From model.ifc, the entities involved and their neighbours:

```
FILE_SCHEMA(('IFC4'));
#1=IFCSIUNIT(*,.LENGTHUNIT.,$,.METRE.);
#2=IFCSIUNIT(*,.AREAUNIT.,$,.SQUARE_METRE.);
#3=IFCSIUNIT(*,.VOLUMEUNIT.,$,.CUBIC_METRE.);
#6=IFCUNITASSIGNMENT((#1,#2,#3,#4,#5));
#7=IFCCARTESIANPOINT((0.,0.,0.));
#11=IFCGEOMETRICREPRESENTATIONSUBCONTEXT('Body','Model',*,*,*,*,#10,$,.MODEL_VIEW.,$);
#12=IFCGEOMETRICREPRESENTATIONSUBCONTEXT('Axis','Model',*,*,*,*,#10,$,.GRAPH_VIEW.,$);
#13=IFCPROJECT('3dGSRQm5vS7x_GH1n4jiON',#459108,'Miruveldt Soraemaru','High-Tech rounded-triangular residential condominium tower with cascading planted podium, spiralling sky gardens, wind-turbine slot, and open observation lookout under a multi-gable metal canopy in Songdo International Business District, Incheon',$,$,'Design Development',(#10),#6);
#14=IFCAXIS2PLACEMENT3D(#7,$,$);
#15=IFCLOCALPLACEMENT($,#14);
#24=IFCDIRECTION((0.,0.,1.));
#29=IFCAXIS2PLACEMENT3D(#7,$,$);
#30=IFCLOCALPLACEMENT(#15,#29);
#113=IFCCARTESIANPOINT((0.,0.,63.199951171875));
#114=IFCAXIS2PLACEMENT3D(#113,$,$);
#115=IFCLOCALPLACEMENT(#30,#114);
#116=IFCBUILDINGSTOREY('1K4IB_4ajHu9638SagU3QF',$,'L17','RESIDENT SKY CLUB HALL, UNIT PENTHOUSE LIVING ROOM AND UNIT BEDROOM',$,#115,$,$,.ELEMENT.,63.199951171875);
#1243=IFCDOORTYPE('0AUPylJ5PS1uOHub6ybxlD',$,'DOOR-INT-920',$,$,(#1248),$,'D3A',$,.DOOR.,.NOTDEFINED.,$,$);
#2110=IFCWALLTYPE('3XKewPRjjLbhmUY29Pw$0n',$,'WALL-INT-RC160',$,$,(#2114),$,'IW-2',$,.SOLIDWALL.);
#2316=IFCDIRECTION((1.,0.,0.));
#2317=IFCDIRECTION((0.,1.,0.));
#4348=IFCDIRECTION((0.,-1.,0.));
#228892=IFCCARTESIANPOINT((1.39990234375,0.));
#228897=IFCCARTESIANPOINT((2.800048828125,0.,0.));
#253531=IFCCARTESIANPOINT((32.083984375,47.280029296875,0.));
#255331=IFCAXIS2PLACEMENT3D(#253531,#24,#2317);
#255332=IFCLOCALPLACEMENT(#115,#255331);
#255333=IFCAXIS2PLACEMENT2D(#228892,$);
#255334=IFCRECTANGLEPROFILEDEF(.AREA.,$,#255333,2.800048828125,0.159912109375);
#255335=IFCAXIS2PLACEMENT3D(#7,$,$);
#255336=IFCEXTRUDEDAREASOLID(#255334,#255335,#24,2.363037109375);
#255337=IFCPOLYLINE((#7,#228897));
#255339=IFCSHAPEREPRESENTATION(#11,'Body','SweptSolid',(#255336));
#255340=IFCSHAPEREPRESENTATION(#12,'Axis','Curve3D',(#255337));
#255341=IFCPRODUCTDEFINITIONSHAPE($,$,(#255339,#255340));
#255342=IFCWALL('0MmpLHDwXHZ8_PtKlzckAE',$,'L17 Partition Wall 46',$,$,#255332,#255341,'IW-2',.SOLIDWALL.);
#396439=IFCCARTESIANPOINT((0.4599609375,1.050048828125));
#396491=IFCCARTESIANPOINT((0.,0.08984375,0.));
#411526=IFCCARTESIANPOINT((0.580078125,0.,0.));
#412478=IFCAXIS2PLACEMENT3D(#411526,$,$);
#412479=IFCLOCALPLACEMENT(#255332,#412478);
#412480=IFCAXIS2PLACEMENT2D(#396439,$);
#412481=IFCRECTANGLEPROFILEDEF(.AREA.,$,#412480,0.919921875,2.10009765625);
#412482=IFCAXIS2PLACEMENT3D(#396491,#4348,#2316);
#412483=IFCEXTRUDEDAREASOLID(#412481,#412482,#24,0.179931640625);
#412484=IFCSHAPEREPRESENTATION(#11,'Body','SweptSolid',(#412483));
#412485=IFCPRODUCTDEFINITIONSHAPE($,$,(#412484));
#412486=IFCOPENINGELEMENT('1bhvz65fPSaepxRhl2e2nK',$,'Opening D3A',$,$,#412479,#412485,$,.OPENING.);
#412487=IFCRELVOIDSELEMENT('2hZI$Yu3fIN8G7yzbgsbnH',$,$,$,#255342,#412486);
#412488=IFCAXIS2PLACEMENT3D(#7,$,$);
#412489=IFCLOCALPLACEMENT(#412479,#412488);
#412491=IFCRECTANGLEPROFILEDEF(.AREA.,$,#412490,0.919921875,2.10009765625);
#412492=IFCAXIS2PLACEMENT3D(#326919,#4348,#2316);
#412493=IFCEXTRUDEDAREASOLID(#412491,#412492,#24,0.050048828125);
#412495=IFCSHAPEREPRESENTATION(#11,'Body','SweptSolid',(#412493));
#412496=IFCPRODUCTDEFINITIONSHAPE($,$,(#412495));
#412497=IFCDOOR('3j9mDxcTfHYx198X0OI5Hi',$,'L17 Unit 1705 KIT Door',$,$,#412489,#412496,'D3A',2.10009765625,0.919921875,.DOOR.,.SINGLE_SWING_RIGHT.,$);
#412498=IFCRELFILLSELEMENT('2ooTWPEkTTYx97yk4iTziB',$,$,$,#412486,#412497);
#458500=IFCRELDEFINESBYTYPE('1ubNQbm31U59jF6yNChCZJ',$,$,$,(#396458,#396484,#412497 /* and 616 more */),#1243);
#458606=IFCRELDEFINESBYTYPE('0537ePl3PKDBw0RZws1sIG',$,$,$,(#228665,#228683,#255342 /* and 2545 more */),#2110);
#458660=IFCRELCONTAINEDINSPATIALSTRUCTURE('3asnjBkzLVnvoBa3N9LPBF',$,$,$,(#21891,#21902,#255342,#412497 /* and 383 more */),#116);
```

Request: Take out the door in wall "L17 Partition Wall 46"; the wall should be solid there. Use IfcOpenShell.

```python
import ifcopenshell
import ifcopenshell.api.feature
import ifcopenshell.api.root
import ifcopenshell.geom
import ifcopenshell.util.shape

model = ifcopenshell.open("model.ifc")
settings = ifcopenshell.geom.settings()


def volume(element):
    """Net volume in cubic metres, openings subtracted."""
    shape = ifcopenshell.geom.create_shape(settings, element)
    return ifcopenshell.util.shape.get_volume(shape.geometry)


door = model.by_guid("3j9mDxcTfHYx198X0OI5Hi")
opening = door.FillsVoids[0].RelatingOpeningElement
wall = opening.VoidsElements[0].RelatingBuildingElement
before = volume(wall)

ifcopenshell.api.root.remove_product(model, product=door)
ifcopenshell.api.feature.remove_feature(model, feature=opening)

after = volume(wall)

print(f"wall volume {before:.3f} -> {after:.3f} m3")

model.write("model_edited.ifc")
```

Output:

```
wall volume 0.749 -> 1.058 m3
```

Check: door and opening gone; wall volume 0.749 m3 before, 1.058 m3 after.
